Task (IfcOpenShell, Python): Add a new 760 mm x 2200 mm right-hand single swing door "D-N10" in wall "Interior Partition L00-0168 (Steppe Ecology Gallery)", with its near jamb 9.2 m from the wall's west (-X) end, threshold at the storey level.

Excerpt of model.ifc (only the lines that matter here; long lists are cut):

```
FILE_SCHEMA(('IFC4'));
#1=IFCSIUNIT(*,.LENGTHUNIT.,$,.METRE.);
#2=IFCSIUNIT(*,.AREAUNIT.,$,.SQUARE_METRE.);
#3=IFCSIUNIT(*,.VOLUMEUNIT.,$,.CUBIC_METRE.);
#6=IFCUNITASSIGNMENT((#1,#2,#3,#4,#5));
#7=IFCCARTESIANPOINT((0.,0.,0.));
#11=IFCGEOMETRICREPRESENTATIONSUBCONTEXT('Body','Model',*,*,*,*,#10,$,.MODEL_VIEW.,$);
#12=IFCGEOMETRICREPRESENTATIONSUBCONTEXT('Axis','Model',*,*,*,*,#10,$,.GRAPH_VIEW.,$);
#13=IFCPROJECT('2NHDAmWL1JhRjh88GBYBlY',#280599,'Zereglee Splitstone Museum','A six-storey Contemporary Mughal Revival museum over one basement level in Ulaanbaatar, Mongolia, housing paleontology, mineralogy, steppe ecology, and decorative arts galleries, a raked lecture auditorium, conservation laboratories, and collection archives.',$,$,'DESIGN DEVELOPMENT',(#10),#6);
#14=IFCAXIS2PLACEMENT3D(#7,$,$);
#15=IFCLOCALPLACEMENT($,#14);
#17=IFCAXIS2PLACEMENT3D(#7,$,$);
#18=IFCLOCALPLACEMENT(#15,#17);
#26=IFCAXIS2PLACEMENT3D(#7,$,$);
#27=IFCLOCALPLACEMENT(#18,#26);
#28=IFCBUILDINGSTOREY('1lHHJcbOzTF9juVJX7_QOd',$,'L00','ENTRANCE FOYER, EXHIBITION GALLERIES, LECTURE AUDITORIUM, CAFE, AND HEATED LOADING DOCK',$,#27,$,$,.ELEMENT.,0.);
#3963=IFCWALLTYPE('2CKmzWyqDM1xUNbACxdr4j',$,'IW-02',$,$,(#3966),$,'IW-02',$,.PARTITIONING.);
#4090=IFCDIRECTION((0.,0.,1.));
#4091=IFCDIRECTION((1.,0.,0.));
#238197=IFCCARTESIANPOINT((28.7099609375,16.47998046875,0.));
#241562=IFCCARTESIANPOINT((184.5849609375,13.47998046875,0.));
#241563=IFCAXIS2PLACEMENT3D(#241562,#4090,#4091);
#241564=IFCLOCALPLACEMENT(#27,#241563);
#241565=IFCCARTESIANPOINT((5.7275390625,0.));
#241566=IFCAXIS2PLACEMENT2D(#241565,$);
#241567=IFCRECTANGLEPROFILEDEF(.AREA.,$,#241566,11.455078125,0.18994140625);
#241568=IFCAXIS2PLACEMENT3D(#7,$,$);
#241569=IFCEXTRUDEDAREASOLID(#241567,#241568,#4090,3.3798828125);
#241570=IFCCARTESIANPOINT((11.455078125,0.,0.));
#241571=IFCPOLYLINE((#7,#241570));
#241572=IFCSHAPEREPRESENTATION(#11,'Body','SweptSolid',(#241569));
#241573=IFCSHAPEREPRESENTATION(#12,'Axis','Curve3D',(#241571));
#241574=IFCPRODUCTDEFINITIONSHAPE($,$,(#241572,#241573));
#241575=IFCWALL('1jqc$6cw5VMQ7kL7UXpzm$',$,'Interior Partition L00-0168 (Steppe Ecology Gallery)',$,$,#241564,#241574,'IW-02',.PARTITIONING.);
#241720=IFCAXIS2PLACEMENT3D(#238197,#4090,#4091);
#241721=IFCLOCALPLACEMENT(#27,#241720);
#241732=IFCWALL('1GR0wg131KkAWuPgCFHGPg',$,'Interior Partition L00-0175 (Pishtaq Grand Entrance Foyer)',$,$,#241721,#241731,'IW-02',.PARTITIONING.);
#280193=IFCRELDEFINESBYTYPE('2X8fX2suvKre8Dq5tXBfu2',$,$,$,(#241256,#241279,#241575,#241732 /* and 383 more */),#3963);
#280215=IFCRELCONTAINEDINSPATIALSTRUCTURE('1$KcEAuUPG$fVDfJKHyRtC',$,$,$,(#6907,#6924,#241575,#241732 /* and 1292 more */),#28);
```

```python
import numpy as np
import ifcopenshell
import ifcopenshell.api.feature
import ifcopenshell.api.geometry
import ifcopenshell.api.root
import ifcopenshell.api.spatial
import ifcopenshell.geom
import ifcopenshell.util.element
import ifcopenshell.util.placement
import ifcopenshell.util.representation
import ifcopenshell.util.shape
import ifcopenshell.util.unit

model = ifcopenshell.open("model.ifc")
unit_scale = ifcopenshell.util.unit.calculate_unit_scale(model)
settings = ifcopenshell.geom.settings()


def volume(element):
    """Net volume in cubic metres, openings subtracted."""
    shape = ifcopenshell.geom.create_shape(settings, element)
    return ifcopenshell.util.shape.get_volume(shape.geometry)


wall = model.by_guid("1jqc$6cw5VMQ7kL7UXpzm$")
storey = ifcopenshell.util.element.get_container(wall, ifc_class="IfcBuildingStorey")
context = ifcopenshell.util.representation.get_context(model, "Model", "Body", "MODEL_VIEW")
before = volume(wall)

width, height, from_end, sill = 0.76, 2.2, 9.2, 0.0  # metres

# The wall runs along its own X axis, and the end named is its -X end.
wall_shape = ifcopenshell.geom.create_shape(settings, wall)
x, y, z = ifcopenshell.util.shape.get_vertices(wall_shape.geometry).T
start = x.min() + from_end
face, thickness = float(y.min()), float(y.max() - y.min())
wall_matrix = ifcopenshell.util.placement.get_local_placement(wall.ObjectPlacement)
level = ifcopenshell.util.placement.get_local_placement(storey.ObjectPlacement)[2, 3]


def in_wall(x, y):
    """Placement at x, y metres in the wall's axes, at sill height."""
    matrix = wall_matrix.copy()
    matrix[:, 3] = wall_matrix @ np.array([x / unit_scale, y / unit_scale, 0.0, 1.0])
    matrix[2, 3] = level + sill / unit_scale
    return matrix


# Opening: a box that overshoots both wall faces by 50 mm.
opening = ifcopenshell.api.root.create_entity(model, ifc_class="IfcOpeningElement", predefined_type="OPENING")
box = ifcopenshell.api.geometry.add_wall_representation(
    model, context=context, length=width, height=height, thickness=thickness + 0.1
)
ifcopenshell.api.geometry.assign_representation(model, product=opening, representation=box)
ifcopenshell.api.geometry.edit_object_placement(model, product=opening, matrix=in_wall(start, face - 0.05), is_si=False)
ifcopenshell.api.feature.add_feature(model, feature=opening, element=wall)

door = ifcopenshell.api.root.create_entity(model, ifc_class="IfcDoor", name="D-N10", predefined_type="DOOR")
door.OverallWidth, door.OverallHeight = width / unit_scale, height / unit_scale
door.OperationType = "SINGLE_SWING_RIGHT"
body = ifcopenshell.api.geometry.add_door_representation(
    model,
    context=context,
    overall_width=door.OverallWidth,
    overall_height=door.OverallHeight,
    operation_type="SINGLE_SWING_RIGHT",
    lining_properties={"LiningDepth": thickness / unit_scale, "ThresholdDepth": thickness / unit_scale},
)
ifcopenshell.api.geometry.assign_representation(model, product=door, representation=body)
ifcopenshell.api.spatial.assign_container(model, products=[door], relating_structure=storey)
ifcopenshell.api.feature.add_filling(model, opening=opening, element=door)

# The lining spans the wall, so the door starts at the wall face.
ifcopenshell.api.geometry.edit_object_placement(model, product=door, matrix=in_wall(start, face), is_si=False)

after = volume(wall)

print(f"wall volume {before:.3f} -> {after:.3f} m3")

model.write("model_v2.ifc")
```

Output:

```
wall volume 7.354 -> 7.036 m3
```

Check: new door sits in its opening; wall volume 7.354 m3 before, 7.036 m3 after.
